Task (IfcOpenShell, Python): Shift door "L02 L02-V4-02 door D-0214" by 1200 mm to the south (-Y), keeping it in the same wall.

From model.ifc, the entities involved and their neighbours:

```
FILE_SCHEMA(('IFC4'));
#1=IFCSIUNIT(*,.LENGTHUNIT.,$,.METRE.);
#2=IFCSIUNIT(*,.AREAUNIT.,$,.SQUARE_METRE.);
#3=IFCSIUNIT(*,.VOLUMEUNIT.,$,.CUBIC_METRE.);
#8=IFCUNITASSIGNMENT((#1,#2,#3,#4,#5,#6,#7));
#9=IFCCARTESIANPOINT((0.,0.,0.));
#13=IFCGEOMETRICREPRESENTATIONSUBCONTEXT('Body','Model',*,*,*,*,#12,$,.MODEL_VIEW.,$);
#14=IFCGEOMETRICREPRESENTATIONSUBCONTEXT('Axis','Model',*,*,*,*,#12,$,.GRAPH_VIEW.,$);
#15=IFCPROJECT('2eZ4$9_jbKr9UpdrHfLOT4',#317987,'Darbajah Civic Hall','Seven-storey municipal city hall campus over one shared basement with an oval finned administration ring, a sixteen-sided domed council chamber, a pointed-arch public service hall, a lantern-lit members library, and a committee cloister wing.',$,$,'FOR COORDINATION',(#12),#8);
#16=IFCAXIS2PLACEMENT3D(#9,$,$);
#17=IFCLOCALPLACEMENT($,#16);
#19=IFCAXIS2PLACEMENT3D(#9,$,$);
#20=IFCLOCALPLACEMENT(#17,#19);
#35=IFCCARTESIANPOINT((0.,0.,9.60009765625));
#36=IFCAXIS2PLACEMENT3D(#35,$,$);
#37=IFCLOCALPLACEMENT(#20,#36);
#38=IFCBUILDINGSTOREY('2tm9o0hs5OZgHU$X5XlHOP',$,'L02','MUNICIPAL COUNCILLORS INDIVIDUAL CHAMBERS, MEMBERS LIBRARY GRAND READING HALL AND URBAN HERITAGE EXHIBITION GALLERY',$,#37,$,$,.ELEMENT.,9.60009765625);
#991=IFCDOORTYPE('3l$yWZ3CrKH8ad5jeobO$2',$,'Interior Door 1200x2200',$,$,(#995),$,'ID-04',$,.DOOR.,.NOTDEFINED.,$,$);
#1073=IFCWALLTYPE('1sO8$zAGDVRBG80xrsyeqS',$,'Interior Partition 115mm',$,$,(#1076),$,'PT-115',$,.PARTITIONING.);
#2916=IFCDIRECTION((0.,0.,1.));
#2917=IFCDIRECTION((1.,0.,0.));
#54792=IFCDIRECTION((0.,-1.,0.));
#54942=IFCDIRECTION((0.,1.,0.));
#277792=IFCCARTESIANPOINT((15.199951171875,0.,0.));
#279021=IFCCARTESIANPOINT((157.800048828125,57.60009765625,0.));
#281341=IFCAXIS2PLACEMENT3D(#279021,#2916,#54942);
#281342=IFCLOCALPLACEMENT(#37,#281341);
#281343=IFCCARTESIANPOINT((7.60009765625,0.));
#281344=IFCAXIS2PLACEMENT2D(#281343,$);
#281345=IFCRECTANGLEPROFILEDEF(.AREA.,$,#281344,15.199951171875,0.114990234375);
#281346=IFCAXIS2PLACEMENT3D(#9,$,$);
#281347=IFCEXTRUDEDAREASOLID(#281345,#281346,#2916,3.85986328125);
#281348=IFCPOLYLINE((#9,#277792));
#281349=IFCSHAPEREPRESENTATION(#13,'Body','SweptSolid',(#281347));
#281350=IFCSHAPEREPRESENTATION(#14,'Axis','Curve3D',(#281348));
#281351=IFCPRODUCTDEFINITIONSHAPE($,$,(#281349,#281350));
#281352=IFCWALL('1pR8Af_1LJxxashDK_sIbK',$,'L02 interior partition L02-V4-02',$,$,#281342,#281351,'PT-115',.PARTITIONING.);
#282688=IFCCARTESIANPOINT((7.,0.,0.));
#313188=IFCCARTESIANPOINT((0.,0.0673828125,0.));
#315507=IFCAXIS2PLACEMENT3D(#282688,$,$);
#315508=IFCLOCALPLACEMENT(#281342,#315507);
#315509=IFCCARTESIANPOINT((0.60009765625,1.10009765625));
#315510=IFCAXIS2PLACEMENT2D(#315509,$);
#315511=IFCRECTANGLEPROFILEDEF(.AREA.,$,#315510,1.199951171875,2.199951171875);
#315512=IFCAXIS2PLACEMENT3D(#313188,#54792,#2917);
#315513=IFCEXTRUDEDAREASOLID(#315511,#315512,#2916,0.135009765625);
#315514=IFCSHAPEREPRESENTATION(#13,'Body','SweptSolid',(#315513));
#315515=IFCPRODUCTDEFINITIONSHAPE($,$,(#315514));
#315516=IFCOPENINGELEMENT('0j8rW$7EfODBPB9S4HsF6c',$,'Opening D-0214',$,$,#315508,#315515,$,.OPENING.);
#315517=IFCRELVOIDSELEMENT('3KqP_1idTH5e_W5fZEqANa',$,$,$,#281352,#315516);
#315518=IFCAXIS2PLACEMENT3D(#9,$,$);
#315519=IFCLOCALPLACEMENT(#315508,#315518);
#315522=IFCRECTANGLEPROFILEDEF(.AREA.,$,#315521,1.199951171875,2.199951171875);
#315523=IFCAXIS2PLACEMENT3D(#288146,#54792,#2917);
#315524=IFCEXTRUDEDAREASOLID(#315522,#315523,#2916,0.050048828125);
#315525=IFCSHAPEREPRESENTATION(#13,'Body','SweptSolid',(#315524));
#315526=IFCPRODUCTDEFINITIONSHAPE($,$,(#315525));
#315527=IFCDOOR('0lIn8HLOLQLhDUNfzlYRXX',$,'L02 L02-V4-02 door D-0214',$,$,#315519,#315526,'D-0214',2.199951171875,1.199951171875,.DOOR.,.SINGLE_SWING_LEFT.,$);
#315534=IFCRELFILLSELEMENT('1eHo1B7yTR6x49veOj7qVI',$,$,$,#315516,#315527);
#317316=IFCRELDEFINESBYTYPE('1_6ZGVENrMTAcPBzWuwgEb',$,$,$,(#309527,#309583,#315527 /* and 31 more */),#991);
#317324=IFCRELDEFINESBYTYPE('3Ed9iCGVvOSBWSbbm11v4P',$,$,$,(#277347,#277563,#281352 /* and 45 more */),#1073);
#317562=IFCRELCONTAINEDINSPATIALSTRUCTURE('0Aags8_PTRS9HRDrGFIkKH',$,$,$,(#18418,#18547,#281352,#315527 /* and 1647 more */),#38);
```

```python
import ifcopenshell
import ifcopenshell.api.geometry
import ifcopenshell.util.placement
import ifcopenshell.util.unit

model = ifcopenshell.open("model.ifc")
unit_scale = ifcopenshell.util.unit.calculate_unit_scale(model)

door = model.by_guid("0lIn8HLOLQLhDUNfzlYRXX")
opening = door.FillsVoids[0].RelatingOpeningElement
wall = opening.VoidsElements[0].RelatingBuildingElement

wall_matrix = ifcopenshell.util.placement.get_local_placement(wall.ObjectPlacement)
shift = wall_matrix[:3, 0] * -1.2 / unit_scale
before = ifcopenshell.util.placement.get_local_placement(door.ObjectPlacement)[:3, 3].copy()

# The door is placed relative to its opening, so it follows when the opening moves.
matrix = ifcopenshell.util.placement.get_local_placement(opening.ObjectPlacement)
matrix[:3, 3] += shift
ifcopenshell.api.geometry.edit_object_placement(
    model, product=opening, matrix=matrix, is_si=False, should_transform_children=True
)

after = ifcopenshell.util.placement.get_local_placement(door.ObjectPlacement)[:3, 3]
print("door moved by", (after - before).round(3) + 0.0)

model.write("model_rev.ifc")
```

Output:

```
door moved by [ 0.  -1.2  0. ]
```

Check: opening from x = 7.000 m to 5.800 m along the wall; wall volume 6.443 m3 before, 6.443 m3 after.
